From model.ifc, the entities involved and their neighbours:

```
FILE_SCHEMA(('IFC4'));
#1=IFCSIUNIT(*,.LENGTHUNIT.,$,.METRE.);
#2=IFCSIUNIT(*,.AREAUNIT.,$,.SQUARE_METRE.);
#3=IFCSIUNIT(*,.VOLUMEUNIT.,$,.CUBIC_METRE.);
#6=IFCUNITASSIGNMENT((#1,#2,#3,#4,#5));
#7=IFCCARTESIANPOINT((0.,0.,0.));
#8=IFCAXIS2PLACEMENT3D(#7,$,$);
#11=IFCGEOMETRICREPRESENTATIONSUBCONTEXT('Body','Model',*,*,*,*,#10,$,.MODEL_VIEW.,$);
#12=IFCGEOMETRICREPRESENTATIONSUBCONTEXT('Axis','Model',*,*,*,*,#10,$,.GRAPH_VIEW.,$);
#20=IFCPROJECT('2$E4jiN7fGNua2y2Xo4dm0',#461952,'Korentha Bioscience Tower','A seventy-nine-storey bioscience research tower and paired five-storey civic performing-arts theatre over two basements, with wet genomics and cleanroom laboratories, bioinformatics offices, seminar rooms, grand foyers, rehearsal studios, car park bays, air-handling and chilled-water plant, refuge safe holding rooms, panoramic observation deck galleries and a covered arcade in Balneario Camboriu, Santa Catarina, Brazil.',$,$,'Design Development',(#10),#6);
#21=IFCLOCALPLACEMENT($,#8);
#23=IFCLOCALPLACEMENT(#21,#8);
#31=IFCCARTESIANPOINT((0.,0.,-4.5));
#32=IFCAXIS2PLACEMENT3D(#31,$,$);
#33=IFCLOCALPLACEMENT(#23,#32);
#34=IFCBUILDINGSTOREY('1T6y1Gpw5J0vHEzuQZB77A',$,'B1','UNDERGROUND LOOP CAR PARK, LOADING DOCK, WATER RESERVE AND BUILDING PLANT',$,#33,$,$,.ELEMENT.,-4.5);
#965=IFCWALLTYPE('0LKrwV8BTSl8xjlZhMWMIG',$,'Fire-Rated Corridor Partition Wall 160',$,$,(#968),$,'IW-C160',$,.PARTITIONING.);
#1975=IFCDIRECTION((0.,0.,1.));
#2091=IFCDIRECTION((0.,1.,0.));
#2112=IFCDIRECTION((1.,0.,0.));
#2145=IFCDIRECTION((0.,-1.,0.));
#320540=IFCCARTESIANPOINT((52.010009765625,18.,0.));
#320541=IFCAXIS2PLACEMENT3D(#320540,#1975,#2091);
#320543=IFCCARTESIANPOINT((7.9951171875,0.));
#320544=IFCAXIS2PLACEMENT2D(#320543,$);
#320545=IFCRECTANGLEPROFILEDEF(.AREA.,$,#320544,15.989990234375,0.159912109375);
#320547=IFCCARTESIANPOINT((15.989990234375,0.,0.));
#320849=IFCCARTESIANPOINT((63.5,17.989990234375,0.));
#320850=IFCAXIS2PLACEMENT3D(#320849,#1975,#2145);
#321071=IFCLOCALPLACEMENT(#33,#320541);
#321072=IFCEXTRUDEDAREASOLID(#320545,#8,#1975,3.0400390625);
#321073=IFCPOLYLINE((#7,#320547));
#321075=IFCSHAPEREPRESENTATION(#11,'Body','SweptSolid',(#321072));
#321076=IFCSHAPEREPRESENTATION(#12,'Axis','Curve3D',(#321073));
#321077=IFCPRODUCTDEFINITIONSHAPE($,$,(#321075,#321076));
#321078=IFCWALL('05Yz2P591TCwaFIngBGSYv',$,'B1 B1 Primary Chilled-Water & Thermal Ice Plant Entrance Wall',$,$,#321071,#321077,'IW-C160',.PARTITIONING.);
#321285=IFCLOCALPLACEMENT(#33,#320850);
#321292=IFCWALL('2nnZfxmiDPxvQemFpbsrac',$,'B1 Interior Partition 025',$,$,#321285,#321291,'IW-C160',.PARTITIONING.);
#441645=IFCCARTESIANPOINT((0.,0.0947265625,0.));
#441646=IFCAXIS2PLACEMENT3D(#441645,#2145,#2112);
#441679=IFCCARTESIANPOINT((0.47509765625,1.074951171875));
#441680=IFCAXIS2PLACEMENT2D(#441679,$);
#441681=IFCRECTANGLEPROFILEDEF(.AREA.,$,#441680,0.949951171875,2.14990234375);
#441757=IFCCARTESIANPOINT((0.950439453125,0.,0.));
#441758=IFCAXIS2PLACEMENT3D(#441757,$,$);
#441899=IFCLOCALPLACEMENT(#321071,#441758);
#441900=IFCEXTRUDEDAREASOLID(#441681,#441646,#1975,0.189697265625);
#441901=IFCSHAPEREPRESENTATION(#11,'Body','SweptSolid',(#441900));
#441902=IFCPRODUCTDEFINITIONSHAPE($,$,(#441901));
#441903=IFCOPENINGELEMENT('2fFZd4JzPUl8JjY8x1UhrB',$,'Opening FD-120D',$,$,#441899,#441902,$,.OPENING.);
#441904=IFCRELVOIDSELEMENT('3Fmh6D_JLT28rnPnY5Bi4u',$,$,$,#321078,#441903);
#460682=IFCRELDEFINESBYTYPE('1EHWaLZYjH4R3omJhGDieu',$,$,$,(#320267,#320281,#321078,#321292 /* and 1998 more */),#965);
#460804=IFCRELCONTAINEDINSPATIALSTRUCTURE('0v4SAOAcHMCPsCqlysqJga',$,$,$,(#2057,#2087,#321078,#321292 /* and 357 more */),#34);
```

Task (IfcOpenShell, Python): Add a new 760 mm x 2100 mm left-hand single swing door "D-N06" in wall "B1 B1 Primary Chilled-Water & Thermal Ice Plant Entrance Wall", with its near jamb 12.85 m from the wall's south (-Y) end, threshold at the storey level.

```python
import numpy as np
import ifcopenshell
import ifcopenshell.api.feature
import ifcopenshell.api.geometry
import ifcopenshell.api.root
import ifcopenshell.api.spatial
import ifcopenshell.geom
import ifcopenshell.util.element
import ifcopenshell.util.placement
import ifcopenshell.util.representation
import ifcopenshell.util.shape
import ifcopenshell.util.unit

model = ifcopenshell.open("model.ifc")
unit_scale = ifcopenshell.util.unit.calculate_unit_scale(model)
settings = ifcopenshell.geom.settings()


def volume(element):
    """Net volume in cubic metres, openings subtracted."""
    shape = ifcopenshell.geom.create_shape(settings, element)
    return ifcopenshell.util.shape.get_volume(shape.geometry)


wall = model.by_id(321078)
storey = ifcopenshell.util.element.get_container(wall, ifc_class="IfcBuildingStorey")
context = ifcopenshell.util.representation.get_context(model, "Model", "Body", "MODEL_VIEW")
before = volume(wall)

width, height, from_end, sill = 0.76, 2.1, 12.85, 0.0  # metres

# The wall runs along its own X axis, and the end named is its -X end.
wall_shape = ifcopenshell.geom.create_shape(settings, wall)
x, y, z = ifcopenshell.util.shape.get_vertices(wall_shape.geometry).T
start = x.min() + from_end
face, thickness = float(y.min()), float(y.max() - y.min())
wall_matrix = ifcopenshell.util.placement.get_local_placement(wall.ObjectPlacement)
level = ifcopenshell.util.placement.get_local_placement(storey.ObjectPlacement)[2, 3]


def in_wall(x, y):
    """Placement at x, y metres in the wall's axes, at sill height."""
    matrix = wall_matrix.copy()
    matrix[:, 3] = wall_matrix @ np.array([x / unit_scale, y / unit_scale, 0.0, 1.0])
    matrix[2, 3] = level + sill / unit_scale
    return matrix


# Opening: a box that overshoots both wall faces by 50 mm.
opening = ifcopenshell.api.root.create_entity(model, ifc_class="IfcOpeningElement", predefined_type="OPENING")
box = ifcopenshell.api.geometry.add_wall_representation(
    model, context=context, length=width, height=height, thickness=thickness + 0.1
)
ifcopenshell.api.geometry.assign_representation(model, product=opening, representation=box)
ifcopenshell.api.geometry.edit_object_placement(model, product=opening, matrix=in_wall(start, face - 0.05), is_si=False)
ifcopenshell.api.feature.add_feature(model, feature=opening, element=wall)

door = ifcopenshell.api.root.create_entity(model, ifc_class="IfcDoor", name="D-N06", predefined_type="DOOR")
door.OverallWidth, door.OverallHeight = width / unit_scale, height / unit_scale
door.OperationType = "SINGLE_SWING_LEFT"
body = ifcopenshell.api.geometry.add_door_representation(
    model,
    context=context,
    overall_width=door.OverallWidth,
    overall_height=door.OverallHeight,
    operation_type="SINGLE_SWING_LEFT",
    lining_properties={"LiningDepth": thickness / unit_scale, "ThresholdDepth": thickness / unit_scale},
)
ifcopenshell.api.geometry.assign_representation(model, product=door, representation=body)
ifcopenshell.api.spatial.assign_container(model, products=[door], relating_structure=storey)
ifcopenshell.api.feature.add_filling(model, opening=opening, element=door)

# The lining spans the wall, so the door starts at the wall face.
ifcopenshell.api.geometry.edit_object_placement(model, product=door, matrix=in_wall(start, face), is_si=False)

after = volume(wall)

print(f"wall volume {before:.3f} -> {after:.3f} m3")

model.write("model_edited.ifc")
```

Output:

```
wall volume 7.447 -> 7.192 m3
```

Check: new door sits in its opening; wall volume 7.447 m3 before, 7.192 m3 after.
